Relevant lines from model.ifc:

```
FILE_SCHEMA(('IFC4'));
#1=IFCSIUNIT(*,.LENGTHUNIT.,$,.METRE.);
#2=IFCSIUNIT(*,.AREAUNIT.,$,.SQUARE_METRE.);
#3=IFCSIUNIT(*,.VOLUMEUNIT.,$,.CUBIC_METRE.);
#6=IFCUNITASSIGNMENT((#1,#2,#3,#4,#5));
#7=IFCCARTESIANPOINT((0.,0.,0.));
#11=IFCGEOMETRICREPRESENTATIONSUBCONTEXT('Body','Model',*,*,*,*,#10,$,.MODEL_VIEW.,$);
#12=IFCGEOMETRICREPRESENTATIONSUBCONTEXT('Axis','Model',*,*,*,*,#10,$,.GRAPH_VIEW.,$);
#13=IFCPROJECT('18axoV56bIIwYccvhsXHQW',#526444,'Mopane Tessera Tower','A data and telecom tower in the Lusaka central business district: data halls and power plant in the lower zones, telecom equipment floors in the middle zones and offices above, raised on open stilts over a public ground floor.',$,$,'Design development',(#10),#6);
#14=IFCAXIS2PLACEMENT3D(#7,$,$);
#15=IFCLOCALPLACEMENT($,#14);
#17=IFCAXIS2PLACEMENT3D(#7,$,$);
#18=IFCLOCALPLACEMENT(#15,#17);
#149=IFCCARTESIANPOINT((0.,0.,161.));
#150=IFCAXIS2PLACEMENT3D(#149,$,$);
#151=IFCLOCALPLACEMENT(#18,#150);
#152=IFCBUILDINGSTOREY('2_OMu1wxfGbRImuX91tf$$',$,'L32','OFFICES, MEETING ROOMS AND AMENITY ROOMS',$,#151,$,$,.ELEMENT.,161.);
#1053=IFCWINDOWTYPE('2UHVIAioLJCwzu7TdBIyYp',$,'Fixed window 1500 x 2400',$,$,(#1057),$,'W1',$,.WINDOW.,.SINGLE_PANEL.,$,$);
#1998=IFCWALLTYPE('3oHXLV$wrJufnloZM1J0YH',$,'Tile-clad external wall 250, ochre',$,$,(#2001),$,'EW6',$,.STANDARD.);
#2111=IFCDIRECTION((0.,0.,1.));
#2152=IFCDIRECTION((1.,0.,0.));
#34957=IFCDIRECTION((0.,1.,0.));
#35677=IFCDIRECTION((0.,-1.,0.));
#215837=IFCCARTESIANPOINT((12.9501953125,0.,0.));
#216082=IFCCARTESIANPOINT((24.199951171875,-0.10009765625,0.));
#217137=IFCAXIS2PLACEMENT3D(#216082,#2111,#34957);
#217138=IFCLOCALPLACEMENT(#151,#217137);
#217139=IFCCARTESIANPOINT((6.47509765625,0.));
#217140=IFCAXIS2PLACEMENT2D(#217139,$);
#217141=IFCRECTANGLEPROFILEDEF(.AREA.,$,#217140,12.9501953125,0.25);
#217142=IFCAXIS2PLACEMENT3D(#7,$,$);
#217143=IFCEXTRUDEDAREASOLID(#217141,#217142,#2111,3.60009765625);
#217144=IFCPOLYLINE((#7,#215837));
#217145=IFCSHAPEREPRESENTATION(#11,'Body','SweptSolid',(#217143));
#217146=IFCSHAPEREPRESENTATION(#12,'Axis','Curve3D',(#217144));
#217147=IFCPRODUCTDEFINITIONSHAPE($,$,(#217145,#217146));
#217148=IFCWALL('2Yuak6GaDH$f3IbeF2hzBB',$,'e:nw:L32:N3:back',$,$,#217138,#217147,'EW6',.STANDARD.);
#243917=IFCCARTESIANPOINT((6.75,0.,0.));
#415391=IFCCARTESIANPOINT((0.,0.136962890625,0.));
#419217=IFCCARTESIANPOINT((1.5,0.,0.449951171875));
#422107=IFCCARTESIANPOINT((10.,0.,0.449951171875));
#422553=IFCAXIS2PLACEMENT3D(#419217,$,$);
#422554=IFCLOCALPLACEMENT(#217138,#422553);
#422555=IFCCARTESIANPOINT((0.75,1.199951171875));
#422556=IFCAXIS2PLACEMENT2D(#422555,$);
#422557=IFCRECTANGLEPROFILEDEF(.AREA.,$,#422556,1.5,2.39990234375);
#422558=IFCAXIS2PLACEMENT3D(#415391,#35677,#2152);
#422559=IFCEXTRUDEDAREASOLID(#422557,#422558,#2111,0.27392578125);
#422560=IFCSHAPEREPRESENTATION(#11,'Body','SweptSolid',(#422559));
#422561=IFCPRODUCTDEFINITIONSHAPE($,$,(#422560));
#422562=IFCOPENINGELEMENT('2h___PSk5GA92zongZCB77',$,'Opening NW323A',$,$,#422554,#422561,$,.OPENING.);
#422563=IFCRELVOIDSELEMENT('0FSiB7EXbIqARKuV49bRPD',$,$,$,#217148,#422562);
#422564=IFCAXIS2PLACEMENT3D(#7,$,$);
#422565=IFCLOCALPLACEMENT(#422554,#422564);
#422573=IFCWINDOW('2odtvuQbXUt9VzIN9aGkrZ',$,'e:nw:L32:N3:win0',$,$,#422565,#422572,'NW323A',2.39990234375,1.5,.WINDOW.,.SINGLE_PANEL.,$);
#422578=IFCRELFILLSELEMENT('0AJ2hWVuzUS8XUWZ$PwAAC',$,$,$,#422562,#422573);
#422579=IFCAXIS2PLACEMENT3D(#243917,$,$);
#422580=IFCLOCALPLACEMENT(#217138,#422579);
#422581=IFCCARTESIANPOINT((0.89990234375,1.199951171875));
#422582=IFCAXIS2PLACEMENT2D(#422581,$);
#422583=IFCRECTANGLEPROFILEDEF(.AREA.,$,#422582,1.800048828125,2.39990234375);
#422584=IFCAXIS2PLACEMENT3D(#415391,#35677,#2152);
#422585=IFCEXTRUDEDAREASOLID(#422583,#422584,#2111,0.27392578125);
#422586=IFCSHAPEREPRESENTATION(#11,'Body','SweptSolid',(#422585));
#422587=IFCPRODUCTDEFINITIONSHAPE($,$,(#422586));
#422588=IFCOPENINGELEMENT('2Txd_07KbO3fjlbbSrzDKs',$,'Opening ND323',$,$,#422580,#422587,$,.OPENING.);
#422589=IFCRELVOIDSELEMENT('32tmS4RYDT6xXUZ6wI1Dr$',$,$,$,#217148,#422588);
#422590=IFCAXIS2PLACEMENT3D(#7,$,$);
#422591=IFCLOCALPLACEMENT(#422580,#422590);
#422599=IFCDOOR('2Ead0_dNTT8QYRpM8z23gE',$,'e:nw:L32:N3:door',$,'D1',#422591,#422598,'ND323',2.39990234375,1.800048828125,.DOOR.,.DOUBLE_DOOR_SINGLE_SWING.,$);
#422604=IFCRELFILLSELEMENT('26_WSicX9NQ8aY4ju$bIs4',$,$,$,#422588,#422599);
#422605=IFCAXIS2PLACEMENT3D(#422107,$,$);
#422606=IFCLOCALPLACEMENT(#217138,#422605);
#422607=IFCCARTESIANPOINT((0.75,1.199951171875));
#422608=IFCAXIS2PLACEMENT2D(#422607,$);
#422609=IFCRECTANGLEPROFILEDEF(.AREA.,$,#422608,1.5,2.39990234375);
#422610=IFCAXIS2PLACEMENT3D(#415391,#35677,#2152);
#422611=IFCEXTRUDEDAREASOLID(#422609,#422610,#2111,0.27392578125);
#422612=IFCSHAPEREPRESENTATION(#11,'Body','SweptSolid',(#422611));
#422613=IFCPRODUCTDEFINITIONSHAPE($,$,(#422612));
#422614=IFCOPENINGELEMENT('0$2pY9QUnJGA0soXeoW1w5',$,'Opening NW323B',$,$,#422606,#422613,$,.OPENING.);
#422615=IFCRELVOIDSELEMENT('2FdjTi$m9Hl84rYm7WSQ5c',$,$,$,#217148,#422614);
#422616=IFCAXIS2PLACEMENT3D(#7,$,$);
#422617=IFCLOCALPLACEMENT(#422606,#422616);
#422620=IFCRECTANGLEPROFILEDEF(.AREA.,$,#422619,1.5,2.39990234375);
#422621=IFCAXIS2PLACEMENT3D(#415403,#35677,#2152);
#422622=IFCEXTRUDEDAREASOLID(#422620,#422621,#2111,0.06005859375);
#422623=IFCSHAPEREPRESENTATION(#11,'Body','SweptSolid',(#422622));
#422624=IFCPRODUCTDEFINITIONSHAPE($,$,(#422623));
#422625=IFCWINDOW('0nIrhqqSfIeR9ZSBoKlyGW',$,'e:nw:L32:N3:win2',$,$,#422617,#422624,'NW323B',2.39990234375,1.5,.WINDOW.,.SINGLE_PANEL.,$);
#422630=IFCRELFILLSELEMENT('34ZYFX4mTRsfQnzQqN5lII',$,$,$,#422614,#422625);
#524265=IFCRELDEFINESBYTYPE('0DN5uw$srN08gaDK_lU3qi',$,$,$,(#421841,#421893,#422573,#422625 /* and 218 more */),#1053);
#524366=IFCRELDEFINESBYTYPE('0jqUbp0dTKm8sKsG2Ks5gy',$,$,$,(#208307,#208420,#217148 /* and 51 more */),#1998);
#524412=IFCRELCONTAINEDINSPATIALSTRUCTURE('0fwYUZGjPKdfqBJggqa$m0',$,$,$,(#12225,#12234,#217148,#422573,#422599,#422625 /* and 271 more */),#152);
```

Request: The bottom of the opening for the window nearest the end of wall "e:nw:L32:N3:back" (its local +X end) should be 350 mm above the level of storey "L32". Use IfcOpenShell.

```python
import numpy as np
import ifcopenshell
import ifcopenshell.api.geometry
import ifcopenshell.geom
import ifcopenshell.util.element
import ifcopenshell.util.placement
import ifcopenshell.util.shape
import ifcopenshell.util.unit

model = ifcopenshell.open("model.ifc")
unit_scale = ifcopenshell.util.unit.calculate_unit_scale(model)

window = model.by_guid("0nIrhqqSfIeR9ZSBoKlyGW")
opening = window.FillsVoids[0].RelatingOpeningElement
storey = ifcopenshell.util.element.get_container(window, ifc_class="IfcBuildingStorey")
level = ifcopenshell.util.placement.get_local_placement(storey.ObjectPlacement)[2, 3]

# The opening's origin need not be at the sill, so measure its lowest point.
shape = ifcopenshell.geom.create_shape(ifcopenshell.geom.settings(), opening)
bottom = ifcopenshell.util.shape.get_shape_bottom_elevation(shape, shape.geometry) / unit_scale
dz = level + 0.35 / unit_scale - bottom

shift = np.array([0.0, 0.0, dz])
# The window is placed relative to its opening, so it follows when the opening moves.
matrix = ifcopenshell.util.placement.get_local_placement(opening.ObjectPlacement)
matrix[:3, 3] += shift
ifcopenshell.api.geometry.edit_object_placement(
    model, product=opening, matrix=matrix, is_si=False, should_transform_children=True
)

print(f"moved by {dz * unit_scale:+.3f} m")

model.write("model-out.ifc")
```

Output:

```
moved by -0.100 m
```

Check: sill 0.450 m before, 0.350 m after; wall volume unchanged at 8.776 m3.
